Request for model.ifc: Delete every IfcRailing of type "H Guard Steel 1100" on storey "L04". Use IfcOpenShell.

First a look at what the model holds.

```python
import ifcopenshell
import ifcopenshell.util.element

model = ifcopenshell.open("model.ifc")
print(model.schema)
storey = next(s for s in model.by_type("IfcBuildingStorey") if s.Name == "L04")
railings = [e for e in ifcopenshell.util.element.get_decomposition(storey) if e.is_a("IfcRailing")]
seen = {}
for e in railings:
    element_type = ifcopenshell.util.element.get_type(e)
    name = element_type.Name if element_type not in (None, e) else None
    seen[name] = seen.get(name, 0) + 1
for name, count in sorted(seen.items(), key=str):
    print(count, "x", name)
```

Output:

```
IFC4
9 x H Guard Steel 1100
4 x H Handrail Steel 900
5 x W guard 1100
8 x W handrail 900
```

```python
import ifcopenshell
import ifcopenshell.api.root
import ifcopenshell.util.element

model = ifcopenshell.open("model.ifc")

storey = next(s for s in model.by_type("IfcBuildingStorey") if s.Name == "L04")
railings = [e for e in ifcopenshell.util.element.get_decomposition(storey) if e.is_a("IfcRailing")]
targets = [e for e in railings if (t := ifcopenshell.util.element.get_type(e)) not in (None, e) and t.Name == "H Guard Steel 1100"]

for e in targets:
    ifcopenshell.api.root.remove_product(model, product=e)
print(len(targets), "removed")

model.write("model_edited.ifc")
```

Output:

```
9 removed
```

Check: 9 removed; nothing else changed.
